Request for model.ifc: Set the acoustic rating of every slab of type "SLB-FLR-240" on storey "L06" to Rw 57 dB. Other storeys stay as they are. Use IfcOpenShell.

First a look at what the model holds.

```python
import ifcopenshell
import ifcopenshell.util.element

model = ifcopenshell.open("model.ifc")
print(model.schema)
storey = next(s for s in model.by_type("IfcBuildingStorey") if s.Name == "L06")
slabs = [e for e in ifcopenshell.util.element.get_decomposition(storey) if e.is_a("IfcSlab")]
seen = {}
for e in slabs:
    element_type = ifcopenshell.util.element.get_type(e)
    key = (element_type.Name if element_type != e and element_type else None, ifcopenshell.util.element.get_pset(e, "Pset_SlabCommon", "AcousticRating"))
    seen[key] = seen.get(key, 0) + 1
for (name, value), count in sorted(seen.items(), key=str):
    print(count, "x", name, "|", value)
```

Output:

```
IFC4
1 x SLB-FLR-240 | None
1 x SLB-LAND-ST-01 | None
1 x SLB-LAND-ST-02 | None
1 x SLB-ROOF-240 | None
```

```python
import ifcopenshell
import ifcopenshell.api.pset
import ifcopenshell.util.element

model = ifcopenshell.open("model.ifc")

storey = next(s for s in model.by_type("IfcBuildingStorey") if s.Name == "L06")
slabs = [e for e in ifcopenshell.util.element.get_decomposition(storey) if e.is_a("IfcSlab")]

count = 0
for e in slabs:
    element_type = ifcopenshell.util.element.get_type(e)
    if element_type in (None, e) or element_type.Name != "SLB-FLR-240":
        continue
    # add_pset returns the element's existing set when there is one.
    pset = ifcopenshell.api.pset.add_pset(model, product=e, name="Pset_SlabCommon")
    ifcopenshell.api.pset.edit_pset(model, pset=pset, properties={"AcousticRating": "Rw 57 dB"})
    count += 1

print(count, "slabs updated")

model.write("model_v2.ifc")
```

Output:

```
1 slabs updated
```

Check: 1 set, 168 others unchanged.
